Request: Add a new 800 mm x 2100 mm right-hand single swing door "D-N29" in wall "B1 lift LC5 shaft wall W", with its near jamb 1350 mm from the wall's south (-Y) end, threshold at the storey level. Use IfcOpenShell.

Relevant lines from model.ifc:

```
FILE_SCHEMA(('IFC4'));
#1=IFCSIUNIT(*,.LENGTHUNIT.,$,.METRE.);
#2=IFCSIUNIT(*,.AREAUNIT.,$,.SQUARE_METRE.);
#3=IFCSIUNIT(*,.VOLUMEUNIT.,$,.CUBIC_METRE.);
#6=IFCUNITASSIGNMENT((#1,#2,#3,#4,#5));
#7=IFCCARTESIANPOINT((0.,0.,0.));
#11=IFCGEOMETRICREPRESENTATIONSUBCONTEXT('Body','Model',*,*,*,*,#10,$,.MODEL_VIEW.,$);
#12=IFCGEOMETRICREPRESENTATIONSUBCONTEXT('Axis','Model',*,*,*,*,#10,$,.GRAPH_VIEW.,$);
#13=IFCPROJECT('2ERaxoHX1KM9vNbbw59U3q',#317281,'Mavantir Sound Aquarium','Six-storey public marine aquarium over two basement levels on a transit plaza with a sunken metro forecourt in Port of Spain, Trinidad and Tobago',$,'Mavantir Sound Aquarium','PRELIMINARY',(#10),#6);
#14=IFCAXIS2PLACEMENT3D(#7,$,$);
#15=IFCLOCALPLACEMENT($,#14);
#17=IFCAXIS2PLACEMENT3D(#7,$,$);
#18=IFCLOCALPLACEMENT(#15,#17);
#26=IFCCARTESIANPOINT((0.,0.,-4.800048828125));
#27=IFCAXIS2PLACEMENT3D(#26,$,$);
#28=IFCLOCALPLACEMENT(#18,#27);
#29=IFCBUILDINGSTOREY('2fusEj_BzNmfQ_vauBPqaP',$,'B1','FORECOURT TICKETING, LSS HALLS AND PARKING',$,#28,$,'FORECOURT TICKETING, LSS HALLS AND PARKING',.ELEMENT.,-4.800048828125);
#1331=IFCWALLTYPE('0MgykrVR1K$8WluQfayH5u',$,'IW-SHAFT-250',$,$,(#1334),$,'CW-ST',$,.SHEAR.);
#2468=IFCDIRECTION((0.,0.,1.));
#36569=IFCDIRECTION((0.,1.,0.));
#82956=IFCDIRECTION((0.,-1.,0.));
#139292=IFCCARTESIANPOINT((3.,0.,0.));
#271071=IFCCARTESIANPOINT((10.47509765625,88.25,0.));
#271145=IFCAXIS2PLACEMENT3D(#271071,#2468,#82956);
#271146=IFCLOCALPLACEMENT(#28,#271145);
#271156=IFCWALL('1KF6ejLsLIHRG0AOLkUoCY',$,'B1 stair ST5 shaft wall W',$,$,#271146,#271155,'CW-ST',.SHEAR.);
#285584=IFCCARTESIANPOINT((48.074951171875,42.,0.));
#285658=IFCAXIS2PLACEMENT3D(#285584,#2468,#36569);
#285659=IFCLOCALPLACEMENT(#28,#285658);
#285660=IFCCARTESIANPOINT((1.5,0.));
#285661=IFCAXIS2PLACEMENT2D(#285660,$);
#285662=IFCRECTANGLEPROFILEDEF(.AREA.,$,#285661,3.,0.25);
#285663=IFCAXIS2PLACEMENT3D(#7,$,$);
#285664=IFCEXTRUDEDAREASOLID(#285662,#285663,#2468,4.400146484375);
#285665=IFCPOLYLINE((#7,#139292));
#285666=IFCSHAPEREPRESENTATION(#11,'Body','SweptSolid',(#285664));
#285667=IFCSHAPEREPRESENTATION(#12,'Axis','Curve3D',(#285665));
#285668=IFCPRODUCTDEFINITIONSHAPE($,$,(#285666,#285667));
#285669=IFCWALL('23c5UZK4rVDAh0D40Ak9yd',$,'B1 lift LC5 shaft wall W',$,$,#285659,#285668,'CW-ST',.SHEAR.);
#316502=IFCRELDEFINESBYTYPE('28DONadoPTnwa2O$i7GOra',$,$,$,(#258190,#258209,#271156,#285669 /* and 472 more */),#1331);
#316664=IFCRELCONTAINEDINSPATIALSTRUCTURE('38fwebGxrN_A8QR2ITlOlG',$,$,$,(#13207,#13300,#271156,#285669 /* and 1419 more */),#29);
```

```python
import numpy as np
import ifcopenshell
import ifcopenshell.api.feature
import ifcopenshell.api.geometry
import ifcopenshell.api.root
import ifcopenshell.api.spatial
import ifcopenshell.geom
import ifcopenshell.util.element
import ifcopenshell.util.placement
import ifcopenshell.util.representation
import ifcopenshell.util.shape
import ifcopenshell.util.unit

model = ifcopenshell.open("model.ifc")
unit_scale = ifcopenshell.util.unit.calculate_unit_scale(model)
settings = ifcopenshell.geom.settings()


def volume(element):
    """Net volume in cubic metres, openings subtracted."""
    shape = ifcopenshell.geom.create_shape(settings, element)
    return ifcopenshell.util.shape.get_volume(shape.geometry)


wall = model.by_id(285669)
storey = ifcopenshell.util.element.get_container(wall, ifc_class="IfcBuildingStorey")
context = ifcopenshell.util.representation.get_context(model, "Model", "Body", "MODEL_VIEW")
before = volume(wall)

width, height, from_end, sill = 0.8, 2.1, 1.35, 0.0  # metres

# The wall runs along its own X axis, and the end named is its -X end.
wall_shape = ifcopenshell.geom.create_shape(settings, wall)
x, y, z = ifcopenshell.util.shape.get_vertices(wall_shape.geometry).T
start = x.min() + from_end
face, thickness = float(y.min()), float(y.max() - y.min())
wall_matrix = ifcopenshell.util.placement.get_local_placement(wall.ObjectPlacement)
level = ifcopenshell.util.placement.get_local_placement(storey.ObjectPlacement)[2, 3]


def in_wall(x, y):
    """Placement at x, y metres in the wall's axes, at sill height."""
    matrix = wall_matrix.copy()
    matrix[:, 3] = wall_matrix @ np.array([x / unit_scale, y / unit_scale, 0.0, 1.0])
    matrix[2, 3] = level + sill / unit_scale
    return matrix


# Opening: a box that overshoots both wall faces by 50 mm.
opening = ifcopenshell.api.root.create_entity(model, ifc_class="IfcOpeningElement", predefined_type="OPENING")
box = ifcopenshell.api.geometry.add_wall_representation(
    model, context=context, length=width, height=height, thickness=thickness + 0.1
)
ifcopenshell.api.geometry.assign_representation(model, product=opening, representation=box)
ifcopenshell.api.geometry.edit_object_placement(model, product=opening, matrix=in_wall(start, face - 0.05), is_si=False)
ifcopenshell.api.feature.add_feature(model, feature=opening, element=wall)

door = ifcopenshell.api.root.create_entity(model, ifc_class="IfcDoor", name="D-N29", predefined_type="DOOR")
door.OverallWidth, door.OverallHeight = width / unit_scale, height / unit_scale
door.OperationType = "SINGLE_SWING_RIGHT"
body = ifcopenshell.api.geometry.add_door_representation(
    model,
    context=context,
    overall_width=door.OverallWidth,
    overall_height=door.OverallHeight,
    operation_type="SINGLE_SWING_RIGHT",
    lining_properties={"LiningDepth": thickness / unit_scale, "ThresholdDepth": thickness / unit_scale},
)
ifcopenshell.api.geometry.assign_representation(model, product=door, representation=body)
ifcopenshell.api.spatial.assign_container(model, products=[door], relating_structure=storey)
ifcopenshell.api.feature.add_filling(model, opening=opening, element=door)

# The lining spans the wall, so the door starts at the wall face.
ifcopenshell.api.geometry.edit_object_placement(model, product=door, matrix=in_wall(start, face), is_si=False)

after = volume(wall)

print(f"wall volume {before:.3f} -> {after:.3f} m3")

model.write("model_v2.ifc")
```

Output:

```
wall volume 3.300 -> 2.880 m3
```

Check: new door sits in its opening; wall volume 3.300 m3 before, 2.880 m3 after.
